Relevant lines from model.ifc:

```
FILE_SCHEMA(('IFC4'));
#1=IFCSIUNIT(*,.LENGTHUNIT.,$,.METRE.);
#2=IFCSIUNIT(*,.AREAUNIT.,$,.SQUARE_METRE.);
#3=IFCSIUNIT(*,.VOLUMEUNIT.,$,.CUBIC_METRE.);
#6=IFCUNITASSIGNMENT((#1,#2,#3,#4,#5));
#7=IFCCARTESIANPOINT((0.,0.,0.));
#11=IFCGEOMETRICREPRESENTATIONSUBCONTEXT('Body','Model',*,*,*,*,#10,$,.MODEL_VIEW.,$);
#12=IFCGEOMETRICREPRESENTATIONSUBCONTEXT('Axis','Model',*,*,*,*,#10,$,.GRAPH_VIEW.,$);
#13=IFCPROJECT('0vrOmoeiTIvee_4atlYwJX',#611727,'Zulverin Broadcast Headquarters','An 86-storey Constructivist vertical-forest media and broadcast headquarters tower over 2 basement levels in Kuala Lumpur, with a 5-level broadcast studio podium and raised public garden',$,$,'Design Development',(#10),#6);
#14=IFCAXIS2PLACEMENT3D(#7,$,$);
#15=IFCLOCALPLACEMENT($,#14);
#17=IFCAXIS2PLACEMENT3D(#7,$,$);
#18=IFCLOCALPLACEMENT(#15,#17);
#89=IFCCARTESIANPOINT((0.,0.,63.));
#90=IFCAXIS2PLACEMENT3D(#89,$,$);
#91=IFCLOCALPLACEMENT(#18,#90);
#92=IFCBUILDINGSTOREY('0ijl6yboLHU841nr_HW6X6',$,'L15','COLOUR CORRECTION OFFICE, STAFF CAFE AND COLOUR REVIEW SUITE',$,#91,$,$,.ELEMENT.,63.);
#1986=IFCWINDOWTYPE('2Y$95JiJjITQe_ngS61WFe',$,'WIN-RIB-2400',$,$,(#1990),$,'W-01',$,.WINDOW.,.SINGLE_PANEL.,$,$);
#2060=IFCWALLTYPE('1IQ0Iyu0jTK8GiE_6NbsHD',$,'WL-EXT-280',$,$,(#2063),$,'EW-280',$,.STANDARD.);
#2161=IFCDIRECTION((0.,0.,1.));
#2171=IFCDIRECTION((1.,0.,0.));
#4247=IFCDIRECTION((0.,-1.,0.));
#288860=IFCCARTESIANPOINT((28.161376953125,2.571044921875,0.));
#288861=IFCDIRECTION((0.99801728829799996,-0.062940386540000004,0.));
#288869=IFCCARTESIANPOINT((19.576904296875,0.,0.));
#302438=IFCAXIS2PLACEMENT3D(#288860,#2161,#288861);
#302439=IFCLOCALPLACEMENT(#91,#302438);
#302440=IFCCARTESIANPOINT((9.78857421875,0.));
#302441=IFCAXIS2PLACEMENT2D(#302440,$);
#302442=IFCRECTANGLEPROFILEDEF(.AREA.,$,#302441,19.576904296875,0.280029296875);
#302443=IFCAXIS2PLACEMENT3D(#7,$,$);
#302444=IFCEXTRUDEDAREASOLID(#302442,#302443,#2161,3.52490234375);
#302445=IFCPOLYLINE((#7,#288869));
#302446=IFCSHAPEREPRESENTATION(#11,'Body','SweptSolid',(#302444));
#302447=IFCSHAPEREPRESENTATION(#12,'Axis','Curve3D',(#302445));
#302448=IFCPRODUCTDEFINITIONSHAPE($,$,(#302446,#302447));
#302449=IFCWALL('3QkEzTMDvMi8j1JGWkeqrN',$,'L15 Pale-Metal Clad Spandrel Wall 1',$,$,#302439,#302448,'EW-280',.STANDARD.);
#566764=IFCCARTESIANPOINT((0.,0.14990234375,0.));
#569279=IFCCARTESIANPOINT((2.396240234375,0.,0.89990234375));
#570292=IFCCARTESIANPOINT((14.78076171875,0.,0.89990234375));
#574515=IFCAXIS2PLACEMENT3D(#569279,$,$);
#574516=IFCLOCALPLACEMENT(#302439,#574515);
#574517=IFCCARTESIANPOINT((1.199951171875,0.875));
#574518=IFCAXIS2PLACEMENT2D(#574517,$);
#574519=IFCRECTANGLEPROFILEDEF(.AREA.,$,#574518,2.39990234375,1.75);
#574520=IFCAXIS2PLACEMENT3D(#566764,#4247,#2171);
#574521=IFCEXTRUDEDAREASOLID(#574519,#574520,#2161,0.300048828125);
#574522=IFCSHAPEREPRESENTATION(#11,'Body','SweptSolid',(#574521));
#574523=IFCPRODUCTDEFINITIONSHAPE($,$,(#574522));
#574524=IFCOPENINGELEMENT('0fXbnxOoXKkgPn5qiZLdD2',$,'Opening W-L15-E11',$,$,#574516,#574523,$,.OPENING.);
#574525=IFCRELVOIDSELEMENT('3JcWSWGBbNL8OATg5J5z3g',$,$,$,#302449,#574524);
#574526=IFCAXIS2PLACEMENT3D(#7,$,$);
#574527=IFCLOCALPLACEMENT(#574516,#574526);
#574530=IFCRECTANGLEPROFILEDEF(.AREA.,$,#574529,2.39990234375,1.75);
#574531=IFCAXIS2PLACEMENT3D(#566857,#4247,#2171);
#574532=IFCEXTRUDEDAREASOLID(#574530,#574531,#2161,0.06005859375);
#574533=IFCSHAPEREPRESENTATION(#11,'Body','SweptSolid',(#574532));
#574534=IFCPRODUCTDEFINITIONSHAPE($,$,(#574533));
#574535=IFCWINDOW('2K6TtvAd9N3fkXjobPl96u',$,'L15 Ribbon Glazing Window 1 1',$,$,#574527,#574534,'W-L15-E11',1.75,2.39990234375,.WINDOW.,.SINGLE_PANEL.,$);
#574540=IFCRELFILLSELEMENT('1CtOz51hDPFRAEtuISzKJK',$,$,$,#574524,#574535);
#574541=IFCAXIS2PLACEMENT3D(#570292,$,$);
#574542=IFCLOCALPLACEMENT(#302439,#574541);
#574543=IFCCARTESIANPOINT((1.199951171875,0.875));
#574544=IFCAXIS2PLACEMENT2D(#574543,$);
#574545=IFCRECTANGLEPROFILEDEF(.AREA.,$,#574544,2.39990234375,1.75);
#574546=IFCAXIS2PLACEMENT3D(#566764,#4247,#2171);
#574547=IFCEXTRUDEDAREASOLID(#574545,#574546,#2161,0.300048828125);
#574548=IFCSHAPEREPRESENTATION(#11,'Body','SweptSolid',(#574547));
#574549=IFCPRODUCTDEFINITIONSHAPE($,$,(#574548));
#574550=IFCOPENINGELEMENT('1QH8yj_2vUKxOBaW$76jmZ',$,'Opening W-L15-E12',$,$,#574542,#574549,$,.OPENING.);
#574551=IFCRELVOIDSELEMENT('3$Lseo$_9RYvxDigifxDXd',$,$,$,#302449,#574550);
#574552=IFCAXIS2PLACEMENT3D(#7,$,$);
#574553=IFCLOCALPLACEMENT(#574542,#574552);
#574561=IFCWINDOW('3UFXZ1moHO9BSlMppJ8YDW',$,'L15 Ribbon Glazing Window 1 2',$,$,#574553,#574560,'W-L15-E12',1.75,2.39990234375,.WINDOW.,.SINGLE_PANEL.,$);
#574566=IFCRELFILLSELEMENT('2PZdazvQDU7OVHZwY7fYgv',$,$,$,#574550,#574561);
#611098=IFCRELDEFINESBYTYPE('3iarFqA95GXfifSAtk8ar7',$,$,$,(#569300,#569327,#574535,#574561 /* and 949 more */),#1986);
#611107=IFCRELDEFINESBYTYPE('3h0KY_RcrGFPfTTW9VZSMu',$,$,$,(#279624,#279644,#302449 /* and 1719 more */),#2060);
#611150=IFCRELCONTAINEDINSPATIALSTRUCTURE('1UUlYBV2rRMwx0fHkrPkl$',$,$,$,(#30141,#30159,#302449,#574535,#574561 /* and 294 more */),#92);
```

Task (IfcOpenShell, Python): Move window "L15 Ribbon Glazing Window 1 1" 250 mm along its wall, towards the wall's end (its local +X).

```python
import ifcopenshell
import ifcopenshell.api.geometry
import ifcopenshell.util.placement
import ifcopenshell.util.unit

model = ifcopenshell.open("model.ifc")
unit_scale = ifcopenshell.util.unit.calculate_unit_scale(model)

window = model.by_guid("2K6TtvAd9N3fkXjobPl96u")
opening = window.FillsVoids[0].RelatingOpeningElement
wall = opening.VoidsElements[0].RelatingBuildingElement

wall_matrix = ifcopenshell.util.placement.get_local_placement(wall.ObjectPlacement)
shift = wall_matrix[:3, 0] * 0.25 / unit_scale
before = ifcopenshell.util.placement.get_local_placement(window.ObjectPlacement)[:3, 3].copy()

# The window is placed relative to its opening, so it follows when the opening moves.
matrix = ifcopenshell.util.placement.get_local_placement(opening.ObjectPlacement)
matrix[:3, 3] += shift
ifcopenshell.api.geometry.edit_object_placement(
    model, product=opening, matrix=matrix, is_si=False, should_transform_children=True
)

after = ifcopenshell.util.placement.get_local_placement(window.ObjectPlacement)[:3, 3]
print("window moved by", (after - before).round(3) + 0.0)

model.write("model-out.ifc")
```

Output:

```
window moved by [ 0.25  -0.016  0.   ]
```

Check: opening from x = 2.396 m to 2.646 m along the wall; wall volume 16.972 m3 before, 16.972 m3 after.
